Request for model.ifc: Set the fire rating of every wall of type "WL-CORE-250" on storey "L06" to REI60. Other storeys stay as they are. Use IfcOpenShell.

First a look at what the model holds.

```python
import ifcopenshell
import ifcopenshell.util.element

model = ifcopenshell.open("model.ifc")
print(model.schema)
storey = next(s for s in model.by_type("IfcBuildingStorey") if s.Name == "L06")
walls = [e for e in ifcopenshell.util.element.get_decomposition(storey) if e.is_a("IfcWall")]
seen = {}
for e in walls:
    element_type = ifcopenshell.util.element.get_type(e)
    key = (element_type.Name if element_type != e and element_type else None, ifcopenshell.util.element.get_pset(e, "Pset_WallCommon", "FireRating"))
    seen[key] = seen.get(key, 0) + 1
for (name, value), count in sorted(seen.items(), key=str):
    print(count, "x", name, "|", value)
```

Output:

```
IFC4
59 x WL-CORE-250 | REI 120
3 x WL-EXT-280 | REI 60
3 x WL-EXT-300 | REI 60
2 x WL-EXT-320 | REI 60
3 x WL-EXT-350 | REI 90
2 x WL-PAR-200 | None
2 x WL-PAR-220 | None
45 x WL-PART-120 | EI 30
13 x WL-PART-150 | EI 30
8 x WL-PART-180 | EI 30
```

```python
import ifcopenshell
import ifcopenshell.api.pset
import ifcopenshell.util.element

model = ifcopenshell.open("model.ifc")

storey = next(s for s in model.by_type("IfcBuildingStorey") if s.Name == "L06")
walls = [e for e in ifcopenshell.util.element.get_decomposition(storey) if e.is_a("IfcWall")]

count = 0
for e in walls:
    element_type = ifcopenshell.util.element.get_type(e)
    if element_type in (None, e) or element_type.Name != "WL-CORE-250":
        continue
    # add_pset returns the element's existing set when there is one.
    pset = ifcopenshell.api.pset.add_pset(model, product=e, name="Pset_WallCommon")
    ifcopenshell.api.pset.edit_pset(model, pset=pset, properties={"FireRating": "REI60"})
    count += 1

print(count, "walls updated")

model.write("model_updated.ifc")
```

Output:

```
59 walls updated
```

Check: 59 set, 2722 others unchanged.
